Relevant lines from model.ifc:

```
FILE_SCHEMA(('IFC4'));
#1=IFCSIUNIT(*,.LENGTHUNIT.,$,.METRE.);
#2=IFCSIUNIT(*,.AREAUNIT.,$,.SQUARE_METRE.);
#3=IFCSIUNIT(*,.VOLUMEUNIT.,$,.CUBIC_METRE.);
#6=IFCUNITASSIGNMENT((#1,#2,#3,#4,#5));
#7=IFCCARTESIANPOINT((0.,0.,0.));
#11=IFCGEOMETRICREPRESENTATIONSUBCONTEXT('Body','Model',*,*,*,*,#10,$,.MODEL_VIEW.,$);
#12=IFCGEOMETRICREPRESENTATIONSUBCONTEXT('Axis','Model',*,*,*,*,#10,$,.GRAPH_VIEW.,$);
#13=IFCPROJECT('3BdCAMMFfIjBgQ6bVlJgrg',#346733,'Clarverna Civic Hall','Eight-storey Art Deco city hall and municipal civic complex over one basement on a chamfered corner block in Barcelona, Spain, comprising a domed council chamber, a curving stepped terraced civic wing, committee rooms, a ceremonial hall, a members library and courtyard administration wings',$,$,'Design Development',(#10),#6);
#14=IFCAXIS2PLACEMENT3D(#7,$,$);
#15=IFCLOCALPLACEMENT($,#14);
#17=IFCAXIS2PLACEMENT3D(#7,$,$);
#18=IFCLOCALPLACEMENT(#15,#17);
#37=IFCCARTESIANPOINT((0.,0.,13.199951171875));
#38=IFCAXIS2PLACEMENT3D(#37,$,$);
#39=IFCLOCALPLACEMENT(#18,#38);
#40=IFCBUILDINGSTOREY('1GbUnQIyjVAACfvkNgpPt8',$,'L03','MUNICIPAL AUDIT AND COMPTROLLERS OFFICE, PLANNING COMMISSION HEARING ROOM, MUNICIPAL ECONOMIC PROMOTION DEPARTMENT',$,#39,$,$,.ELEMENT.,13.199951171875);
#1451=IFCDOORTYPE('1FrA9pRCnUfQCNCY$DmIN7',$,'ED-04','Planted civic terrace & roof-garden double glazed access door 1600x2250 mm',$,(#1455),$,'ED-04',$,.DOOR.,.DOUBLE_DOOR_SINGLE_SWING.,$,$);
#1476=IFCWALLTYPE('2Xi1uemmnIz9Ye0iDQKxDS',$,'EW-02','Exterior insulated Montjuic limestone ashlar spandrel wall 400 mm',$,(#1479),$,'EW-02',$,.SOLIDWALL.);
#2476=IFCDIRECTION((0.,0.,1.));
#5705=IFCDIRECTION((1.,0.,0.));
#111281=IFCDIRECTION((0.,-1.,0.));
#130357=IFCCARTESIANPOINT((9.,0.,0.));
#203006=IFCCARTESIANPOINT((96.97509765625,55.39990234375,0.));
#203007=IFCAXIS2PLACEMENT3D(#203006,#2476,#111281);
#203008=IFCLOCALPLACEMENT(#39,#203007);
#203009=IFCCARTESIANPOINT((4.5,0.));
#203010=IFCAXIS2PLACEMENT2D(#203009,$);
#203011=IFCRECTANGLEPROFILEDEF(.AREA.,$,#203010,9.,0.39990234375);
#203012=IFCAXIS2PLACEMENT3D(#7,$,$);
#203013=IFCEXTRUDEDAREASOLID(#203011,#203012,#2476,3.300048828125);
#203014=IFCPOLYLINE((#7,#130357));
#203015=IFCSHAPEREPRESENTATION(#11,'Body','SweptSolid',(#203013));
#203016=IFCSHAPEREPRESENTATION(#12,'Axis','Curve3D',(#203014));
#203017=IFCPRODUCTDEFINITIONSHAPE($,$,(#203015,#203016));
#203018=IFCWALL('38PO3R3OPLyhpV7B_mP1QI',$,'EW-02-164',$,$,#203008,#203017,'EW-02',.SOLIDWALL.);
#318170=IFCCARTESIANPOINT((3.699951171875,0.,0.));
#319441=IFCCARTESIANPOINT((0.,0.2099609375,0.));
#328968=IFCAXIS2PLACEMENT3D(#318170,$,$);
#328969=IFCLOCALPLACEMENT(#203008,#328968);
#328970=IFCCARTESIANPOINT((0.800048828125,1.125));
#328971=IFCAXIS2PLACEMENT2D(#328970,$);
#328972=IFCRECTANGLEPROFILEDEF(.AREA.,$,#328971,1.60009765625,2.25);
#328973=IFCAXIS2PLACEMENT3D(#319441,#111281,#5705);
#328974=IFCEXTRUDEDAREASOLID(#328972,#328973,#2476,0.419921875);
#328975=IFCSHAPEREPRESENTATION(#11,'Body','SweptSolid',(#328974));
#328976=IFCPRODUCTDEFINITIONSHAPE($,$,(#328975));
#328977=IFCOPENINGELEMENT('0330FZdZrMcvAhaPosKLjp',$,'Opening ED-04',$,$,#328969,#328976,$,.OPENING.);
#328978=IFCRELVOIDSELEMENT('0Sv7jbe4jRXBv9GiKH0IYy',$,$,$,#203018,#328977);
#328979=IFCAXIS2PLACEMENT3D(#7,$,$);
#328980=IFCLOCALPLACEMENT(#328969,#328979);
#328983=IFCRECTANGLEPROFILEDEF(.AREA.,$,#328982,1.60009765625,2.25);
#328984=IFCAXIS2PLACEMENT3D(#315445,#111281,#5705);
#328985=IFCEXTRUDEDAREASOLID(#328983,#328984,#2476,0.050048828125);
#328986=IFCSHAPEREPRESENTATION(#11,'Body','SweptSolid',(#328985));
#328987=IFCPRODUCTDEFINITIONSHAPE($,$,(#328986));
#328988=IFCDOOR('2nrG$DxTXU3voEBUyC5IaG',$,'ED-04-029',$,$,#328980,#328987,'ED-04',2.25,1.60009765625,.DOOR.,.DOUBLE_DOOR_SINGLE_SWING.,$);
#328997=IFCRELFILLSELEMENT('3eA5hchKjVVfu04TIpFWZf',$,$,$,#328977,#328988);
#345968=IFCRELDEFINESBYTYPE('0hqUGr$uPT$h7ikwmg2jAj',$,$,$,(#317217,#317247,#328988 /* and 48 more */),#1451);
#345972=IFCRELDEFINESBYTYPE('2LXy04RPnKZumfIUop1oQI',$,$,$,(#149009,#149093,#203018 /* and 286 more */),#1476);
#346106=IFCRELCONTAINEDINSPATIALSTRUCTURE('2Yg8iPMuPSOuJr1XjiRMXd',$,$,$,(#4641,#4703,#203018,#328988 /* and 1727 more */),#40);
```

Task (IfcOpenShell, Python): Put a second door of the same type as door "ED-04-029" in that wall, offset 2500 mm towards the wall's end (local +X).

```python
import ifcopenshell
import ifcopenshell.api.feature
import ifcopenshell.api.geometry
import ifcopenshell.api.root
import ifcopenshell.geom
import ifcopenshell.util.element
import ifcopenshell.util.placement
import ifcopenshell.util.shape
import ifcopenshell.util.unit

model = ifcopenshell.open("model.ifc")
unit_scale = ifcopenshell.util.unit.calculate_unit_scale(model)
settings = ifcopenshell.geom.settings()


def volume(element):
    """Net volume in cubic metres, openings subtracted."""
    shape = ifcopenshell.geom.create_shape(settings, element)
    return ifcopenshell.util.shape.get_volume(shape.geometry)


door = model.by_guid("2nrG$DxTXU3voEBUyC5IaG")
opening = door.FillsVoids[0].RelatingOpeningElement
wall = opening.VoidsElements[0].RelatingBuildingElement
before = volume(wall)
shift = ifcopenshell.util.placement.get_local_placement(wall.ObjectPlacement)[:3, 0] * 2.5 / unit_scale

# copy_class copies the void relationship, type, container and properties, but no geometry.
new_opening = ifcopenshell.api.root.copy_class(model, product=opening)
new_opening.Representation = ifcopenshell.util.element.copy_deep(
    model, opening.Representation, exclude=["IfcGeometricRepresentationContext", "IfcRepresentationMap"]
)
new_door = ifcopenshell.api.root.copy_class(model, product=door)
new_door.Representation = ifcopenshell.util.element.copy_deep(
    model, door.Representation, exclude=["IfcGeometricRepresentationContext", "IfcRepresentationMap"]
)
new_door.Tag = None
ifcopenshell.api.feature.add_filling(model, opening=new_opening, element=new_door)

for old, new in ((opening, new_opening), (door, new_door)):
    matrix = ifcopenshell.util.placement.get_local_placement(old.ObjectPlacement)
    matrix[:3, 3] += shift
    ifcopenshell.api.geometry.edit_object_placement(model, product=new, matrix=matrix, is_si=False)

after = volume(wall)

print(f"wall volume {before:.3f} -> {after:.3f} m3")

model.write("model_updated.ifc")
```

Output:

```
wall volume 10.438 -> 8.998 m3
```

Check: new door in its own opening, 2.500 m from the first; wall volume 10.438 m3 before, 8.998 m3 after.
